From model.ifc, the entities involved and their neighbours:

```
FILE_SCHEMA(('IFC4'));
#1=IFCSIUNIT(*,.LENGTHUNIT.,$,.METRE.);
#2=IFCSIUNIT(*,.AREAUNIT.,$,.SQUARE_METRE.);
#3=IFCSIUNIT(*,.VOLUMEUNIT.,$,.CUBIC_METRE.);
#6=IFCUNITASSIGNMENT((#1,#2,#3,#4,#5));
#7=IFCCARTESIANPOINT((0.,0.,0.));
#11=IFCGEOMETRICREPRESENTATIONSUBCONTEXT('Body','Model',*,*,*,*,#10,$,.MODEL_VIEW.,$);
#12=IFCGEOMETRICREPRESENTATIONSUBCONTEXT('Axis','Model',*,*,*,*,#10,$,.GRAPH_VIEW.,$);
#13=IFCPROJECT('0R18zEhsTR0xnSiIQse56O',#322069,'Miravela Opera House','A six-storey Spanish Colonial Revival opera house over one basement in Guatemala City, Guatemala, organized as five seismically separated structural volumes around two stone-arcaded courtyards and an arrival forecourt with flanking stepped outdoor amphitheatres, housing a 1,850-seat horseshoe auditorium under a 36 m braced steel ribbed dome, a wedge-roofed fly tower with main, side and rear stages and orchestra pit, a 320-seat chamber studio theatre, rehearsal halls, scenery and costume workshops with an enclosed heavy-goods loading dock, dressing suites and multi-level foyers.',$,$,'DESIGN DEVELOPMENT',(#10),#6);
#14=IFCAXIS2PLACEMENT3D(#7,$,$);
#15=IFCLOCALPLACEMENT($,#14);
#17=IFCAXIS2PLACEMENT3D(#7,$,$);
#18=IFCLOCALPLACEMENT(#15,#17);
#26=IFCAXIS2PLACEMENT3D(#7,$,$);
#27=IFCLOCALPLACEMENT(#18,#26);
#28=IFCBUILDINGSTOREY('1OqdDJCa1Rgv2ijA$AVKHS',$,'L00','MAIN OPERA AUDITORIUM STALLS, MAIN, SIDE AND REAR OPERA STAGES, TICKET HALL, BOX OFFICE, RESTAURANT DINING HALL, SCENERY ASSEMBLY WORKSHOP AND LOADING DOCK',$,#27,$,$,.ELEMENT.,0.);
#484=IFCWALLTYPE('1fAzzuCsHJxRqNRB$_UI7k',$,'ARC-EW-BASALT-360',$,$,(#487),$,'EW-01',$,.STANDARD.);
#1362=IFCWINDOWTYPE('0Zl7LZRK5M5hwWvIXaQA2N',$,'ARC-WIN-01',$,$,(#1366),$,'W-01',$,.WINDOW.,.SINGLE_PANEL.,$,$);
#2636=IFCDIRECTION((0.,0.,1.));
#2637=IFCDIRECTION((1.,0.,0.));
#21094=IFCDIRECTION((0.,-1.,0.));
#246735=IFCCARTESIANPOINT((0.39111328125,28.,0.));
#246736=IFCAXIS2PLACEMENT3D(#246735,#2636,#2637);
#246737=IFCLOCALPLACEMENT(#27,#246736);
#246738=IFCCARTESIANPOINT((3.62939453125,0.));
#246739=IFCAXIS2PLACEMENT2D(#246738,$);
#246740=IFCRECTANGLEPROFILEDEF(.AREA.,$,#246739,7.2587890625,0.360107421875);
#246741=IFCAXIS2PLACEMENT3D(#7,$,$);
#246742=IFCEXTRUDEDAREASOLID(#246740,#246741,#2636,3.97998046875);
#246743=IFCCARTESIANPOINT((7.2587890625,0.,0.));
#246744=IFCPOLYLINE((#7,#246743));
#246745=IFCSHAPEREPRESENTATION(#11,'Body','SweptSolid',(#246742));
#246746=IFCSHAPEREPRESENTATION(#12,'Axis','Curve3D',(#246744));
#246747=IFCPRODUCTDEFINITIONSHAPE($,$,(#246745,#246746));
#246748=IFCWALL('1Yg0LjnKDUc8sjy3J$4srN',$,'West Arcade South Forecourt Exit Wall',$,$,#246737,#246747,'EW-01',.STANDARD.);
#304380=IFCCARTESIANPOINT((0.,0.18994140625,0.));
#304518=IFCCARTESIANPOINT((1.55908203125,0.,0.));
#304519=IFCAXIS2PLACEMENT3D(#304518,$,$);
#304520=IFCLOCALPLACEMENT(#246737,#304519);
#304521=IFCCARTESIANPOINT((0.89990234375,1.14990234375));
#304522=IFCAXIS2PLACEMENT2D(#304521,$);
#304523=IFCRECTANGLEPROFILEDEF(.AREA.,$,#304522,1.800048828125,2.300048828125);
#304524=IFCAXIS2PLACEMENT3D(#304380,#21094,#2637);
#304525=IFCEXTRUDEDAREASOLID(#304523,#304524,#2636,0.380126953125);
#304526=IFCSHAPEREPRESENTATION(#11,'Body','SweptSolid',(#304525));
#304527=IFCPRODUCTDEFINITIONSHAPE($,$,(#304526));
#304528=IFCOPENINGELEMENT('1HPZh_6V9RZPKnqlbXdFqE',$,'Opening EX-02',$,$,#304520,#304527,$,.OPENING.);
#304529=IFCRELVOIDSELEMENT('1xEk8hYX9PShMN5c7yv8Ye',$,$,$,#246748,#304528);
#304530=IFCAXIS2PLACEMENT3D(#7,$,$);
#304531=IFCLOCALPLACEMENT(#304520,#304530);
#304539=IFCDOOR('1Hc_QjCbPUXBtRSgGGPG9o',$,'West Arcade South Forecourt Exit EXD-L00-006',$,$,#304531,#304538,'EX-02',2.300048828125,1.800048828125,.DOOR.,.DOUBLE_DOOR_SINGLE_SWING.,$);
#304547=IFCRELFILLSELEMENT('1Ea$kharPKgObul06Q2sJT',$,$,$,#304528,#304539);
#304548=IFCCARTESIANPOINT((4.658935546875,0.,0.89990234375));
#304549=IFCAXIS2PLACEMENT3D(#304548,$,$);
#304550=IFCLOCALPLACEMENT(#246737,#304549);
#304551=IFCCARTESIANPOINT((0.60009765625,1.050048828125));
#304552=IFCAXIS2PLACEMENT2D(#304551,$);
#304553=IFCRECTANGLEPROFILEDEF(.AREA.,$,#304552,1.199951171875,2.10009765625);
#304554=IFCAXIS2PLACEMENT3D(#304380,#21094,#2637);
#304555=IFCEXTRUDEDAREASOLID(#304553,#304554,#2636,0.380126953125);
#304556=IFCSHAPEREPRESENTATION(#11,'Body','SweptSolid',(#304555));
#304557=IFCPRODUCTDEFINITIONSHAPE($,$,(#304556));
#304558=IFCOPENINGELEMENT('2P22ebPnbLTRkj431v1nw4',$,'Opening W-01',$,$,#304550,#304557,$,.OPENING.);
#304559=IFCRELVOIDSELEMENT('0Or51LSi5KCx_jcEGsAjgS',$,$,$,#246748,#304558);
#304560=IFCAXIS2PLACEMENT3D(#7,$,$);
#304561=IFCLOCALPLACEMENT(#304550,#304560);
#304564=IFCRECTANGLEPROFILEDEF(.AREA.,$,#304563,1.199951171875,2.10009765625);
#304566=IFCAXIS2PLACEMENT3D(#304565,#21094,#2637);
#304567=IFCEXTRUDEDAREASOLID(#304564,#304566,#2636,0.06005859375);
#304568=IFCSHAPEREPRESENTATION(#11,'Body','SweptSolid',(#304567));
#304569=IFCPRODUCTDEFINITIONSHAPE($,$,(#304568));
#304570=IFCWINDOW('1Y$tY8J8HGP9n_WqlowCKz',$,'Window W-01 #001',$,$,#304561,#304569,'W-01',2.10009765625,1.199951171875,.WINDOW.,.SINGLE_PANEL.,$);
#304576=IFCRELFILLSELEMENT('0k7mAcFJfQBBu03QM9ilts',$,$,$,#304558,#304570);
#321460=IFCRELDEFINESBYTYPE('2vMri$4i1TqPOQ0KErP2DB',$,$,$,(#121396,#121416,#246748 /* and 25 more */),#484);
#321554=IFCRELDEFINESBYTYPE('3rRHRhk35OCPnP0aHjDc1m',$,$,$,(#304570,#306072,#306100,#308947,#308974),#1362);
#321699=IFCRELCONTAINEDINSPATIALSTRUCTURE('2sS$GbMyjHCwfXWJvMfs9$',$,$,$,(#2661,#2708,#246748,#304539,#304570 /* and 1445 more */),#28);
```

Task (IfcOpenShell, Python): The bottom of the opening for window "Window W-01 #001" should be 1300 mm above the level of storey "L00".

```python
import numpy as np
import ifcopenshell
import ifcopenshell.api.geometry
import ifcopenshell.geom
import ifcopenshell.util.element
import ifcopenshell.util.placement
import ifcopenshell.util.shape
import ifcopenshell.util.unit

model = ifcopenshell.open("model.ifc")
unit_scale = ifcopenshell.util.unit.calculate_unit_scale(model)

window = model.by_id(304570)
opening = window.FillsVoids[0].RelatingOpeningElement
storey = ifcopenshell.util.element.get_container(window, ifc_class="IfcBuildingStorey")
level = ifcopenshell.util.placement.get_local_placement(storey.ObjectPlacement)[2, 3]

# The opening's origin need not be at the sill, so measure its lowest point.
shape = ifcopenshell.geom.create_shape(ifcopenshell.geom.settings(), opening)
bottom = ifcopenshell.util.shape.get_shape_bottom_elevation(shape, shape.geometry) / unit_scale
dz = level + 1.3 - bottom

shift = np.array([0.0, 0.0, dz])
# The window is placed relative to its opening, so it follows when the opening moves.
matrix = ifcopenshell.util.placement.get_local_placement(opening.ObjectPlacement)
matrix[:3, 3] += shift
ifcopenshell.api.geometry.edit_object_placement(
    model, product=opening, matrix=matrix, is_si=False, should_transform_children=True
)

print(f"moved by {dz * unit_scale:+.3f} m")

model.write("model_rev.ifc")
```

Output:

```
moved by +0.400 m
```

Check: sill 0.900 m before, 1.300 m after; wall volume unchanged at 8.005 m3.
